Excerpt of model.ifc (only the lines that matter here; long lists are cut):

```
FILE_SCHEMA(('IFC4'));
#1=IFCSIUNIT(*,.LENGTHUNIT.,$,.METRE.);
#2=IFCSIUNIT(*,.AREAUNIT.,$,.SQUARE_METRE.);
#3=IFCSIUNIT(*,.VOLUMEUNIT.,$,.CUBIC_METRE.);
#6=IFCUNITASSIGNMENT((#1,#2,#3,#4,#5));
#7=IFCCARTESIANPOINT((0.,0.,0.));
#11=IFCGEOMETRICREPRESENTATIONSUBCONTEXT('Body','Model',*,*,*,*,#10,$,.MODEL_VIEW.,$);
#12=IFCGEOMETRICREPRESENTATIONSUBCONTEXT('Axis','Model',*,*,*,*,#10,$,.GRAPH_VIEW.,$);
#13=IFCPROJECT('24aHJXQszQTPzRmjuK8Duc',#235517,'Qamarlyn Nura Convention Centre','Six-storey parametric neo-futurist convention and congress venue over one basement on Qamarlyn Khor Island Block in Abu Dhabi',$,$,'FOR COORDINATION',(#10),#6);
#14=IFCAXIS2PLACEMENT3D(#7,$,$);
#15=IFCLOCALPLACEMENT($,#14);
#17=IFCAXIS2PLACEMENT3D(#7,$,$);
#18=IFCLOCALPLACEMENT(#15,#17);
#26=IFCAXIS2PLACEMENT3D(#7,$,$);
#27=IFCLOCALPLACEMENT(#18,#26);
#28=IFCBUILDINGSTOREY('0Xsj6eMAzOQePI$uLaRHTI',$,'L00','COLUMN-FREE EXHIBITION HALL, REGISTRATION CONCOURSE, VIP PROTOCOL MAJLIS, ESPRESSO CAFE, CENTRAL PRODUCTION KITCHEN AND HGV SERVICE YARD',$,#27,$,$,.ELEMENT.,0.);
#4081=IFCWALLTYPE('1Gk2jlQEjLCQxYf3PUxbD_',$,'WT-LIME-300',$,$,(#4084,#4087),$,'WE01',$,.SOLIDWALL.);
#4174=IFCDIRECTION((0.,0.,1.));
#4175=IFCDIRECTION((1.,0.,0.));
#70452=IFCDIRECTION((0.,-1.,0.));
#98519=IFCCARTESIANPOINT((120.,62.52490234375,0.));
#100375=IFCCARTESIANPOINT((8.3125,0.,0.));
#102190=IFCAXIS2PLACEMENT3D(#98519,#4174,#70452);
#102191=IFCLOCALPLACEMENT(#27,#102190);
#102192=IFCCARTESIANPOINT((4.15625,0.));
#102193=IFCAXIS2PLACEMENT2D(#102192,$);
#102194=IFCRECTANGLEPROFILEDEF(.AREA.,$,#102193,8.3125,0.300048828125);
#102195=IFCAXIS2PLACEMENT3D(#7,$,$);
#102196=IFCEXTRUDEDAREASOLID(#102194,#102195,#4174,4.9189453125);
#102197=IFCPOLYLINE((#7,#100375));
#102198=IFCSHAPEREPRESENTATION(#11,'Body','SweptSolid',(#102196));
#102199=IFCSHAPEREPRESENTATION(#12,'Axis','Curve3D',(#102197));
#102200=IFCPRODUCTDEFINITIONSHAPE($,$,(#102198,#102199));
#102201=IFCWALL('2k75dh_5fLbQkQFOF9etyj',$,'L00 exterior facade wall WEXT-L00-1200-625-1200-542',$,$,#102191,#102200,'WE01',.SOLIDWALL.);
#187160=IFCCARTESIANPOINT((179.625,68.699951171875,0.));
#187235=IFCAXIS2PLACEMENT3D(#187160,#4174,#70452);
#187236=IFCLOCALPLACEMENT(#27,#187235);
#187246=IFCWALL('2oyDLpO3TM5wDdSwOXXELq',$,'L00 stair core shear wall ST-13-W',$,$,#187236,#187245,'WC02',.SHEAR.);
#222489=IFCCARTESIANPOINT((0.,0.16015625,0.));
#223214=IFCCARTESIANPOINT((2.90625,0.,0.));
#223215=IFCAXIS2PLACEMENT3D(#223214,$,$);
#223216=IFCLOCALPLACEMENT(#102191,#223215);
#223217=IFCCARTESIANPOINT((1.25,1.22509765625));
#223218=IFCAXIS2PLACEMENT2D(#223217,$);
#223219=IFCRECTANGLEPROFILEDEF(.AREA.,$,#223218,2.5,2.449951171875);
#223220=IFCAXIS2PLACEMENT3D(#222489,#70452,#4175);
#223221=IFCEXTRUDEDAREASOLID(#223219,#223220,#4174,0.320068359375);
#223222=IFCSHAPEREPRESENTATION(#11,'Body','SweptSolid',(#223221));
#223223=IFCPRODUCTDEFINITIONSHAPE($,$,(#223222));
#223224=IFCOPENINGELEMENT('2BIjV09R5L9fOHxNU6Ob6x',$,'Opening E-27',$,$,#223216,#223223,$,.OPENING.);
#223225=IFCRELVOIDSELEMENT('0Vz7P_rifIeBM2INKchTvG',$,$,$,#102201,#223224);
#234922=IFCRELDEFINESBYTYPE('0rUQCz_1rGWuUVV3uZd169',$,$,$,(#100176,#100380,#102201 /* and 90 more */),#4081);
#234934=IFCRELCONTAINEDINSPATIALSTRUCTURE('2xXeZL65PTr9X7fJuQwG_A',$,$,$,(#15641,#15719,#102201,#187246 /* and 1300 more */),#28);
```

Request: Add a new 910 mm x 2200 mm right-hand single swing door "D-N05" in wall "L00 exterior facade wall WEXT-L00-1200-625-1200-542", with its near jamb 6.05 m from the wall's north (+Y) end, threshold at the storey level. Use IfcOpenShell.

```python
import numpy as np
import ifcopenshell
import ifcopenshell.api.feature
import ifcopenshell.api.geometry
import ifcopenshell.api.root
import ifcopenshell.api.spatial
import ifcopenshell.geom
import ifcopenshell.util.element
import ifcopenshell.util.placement
import ifcopenshell.util.representation
import ifcopenshell.util.shape
import ifcopenshell.util.unit

model = ifcopenshell.open("model.ifc")
unit_scale = ifcopenshell.util.unit.calculate_unit_scale(model)
settings = ifcopenshell.geom.settings()


def volume(element):
    """Net volume in cubic metres, openings subtracted."""
    shape = ifcopenshell.geom.create_shape(settings, element)
    return ifcopenshell.util.shape.get_volume(shape.geometry)


wall = model.by_id(102201)
storey = ifcopenshell.util.element.get_container(wall, ifc_class="IfcBuildingStorey")
context = ifcopenshell.util.representation.get_context(model, "Model", "Body", "MODEL_VIEW")
before = volume(wall)

width, height, from_end, sill = 0.91, 2.2, 6.05, 0.0  # metres

# The wall runs along its own X axis, and the end named is its -X end.
wall_shape = ifcopenshell.geom.create_shape(settings, wall)
x, y, z = ifcopenshell.util.shape.get_vertices(wall_shape.geometry).T
start = x.min() + from_end
face, thickness = float(y.min()), float(y.max() - y.min())
wall_matrix = ifcopenshell.util.placement.get_local_placement(wall.ObjectPlacement)
level = ifcopenshell.util.placement.get_local_placement(storey.ObjectPlacement)[2, 3]


def in_wall(x, y):
    """Placement at x, y metres in the wall's axes, at sill height."""
    matrix = wall_matrix.copy()
    matrix[:, 3] = wall_matrix @ np.array([x / unit_scale, y / unit_scale, 0.0, 1.0])
    matrix[2, 3] = level + sill / unit_scale
    return matrix


# Opening: a box that overshoots both wall faces by 50 mm.
opening = ifcopenshell.api.root.create_entity(model, ifc_class="IfcOpeningElement", predefined_type="OPENING")
box = ifcopenshell.api.geometry.add_wall_representation(
    model, context=context, length=width, height=height, thickness=thickness + 0.1
)
ifcopenshell.api.geometry.assign_representation(model, product=opening, representation=box)
ifcopenshell.api.geometry.edit_object_placement(model, product=opening, matrix=in_wall(start, face - 0.05), is_si=False)
ifcopenshell.api.feature.add_feature(model, feature=opening, element=wall)

door = ifcopenshell.api.root.create_entity(model, ifc_class="IfcDoor", name="D-N05", predefined_type="DOOR")
door.OverallWidth, door.OverallHeight = width / unit_scale, height / unit_scale
door.OperationType = "SINGLE_SWING_RIGHT"
body = ifcopenshell.api.geometry.add_door_representation(
    model,
    context=context,
    overall_width=door.OverallWidth,
    overall_height=door.OverallHeight,
    operation_type="SINGLE_SWING_RIGHT",
    lining_properties={"LiningDepth": thickness / unit_scale, "ThresholdDepth": thickness / unit_scale},
)
ifcopenshell.api.geometry.assign_representation(model, product=door, representation=body)
ifcopenshell.api.spatial.assign_container(model, products=[door], relating_structure=storey)
ifcopenshell.api.feature.add_filling(model, opening=opening, element=door)

# The lining spans the wall, so the door starts at the wall face.
ifcopenshell.api.geometry.edit_object_placement(model, product=door, matrix=in_wall(start, face), is_si=False)

after = volume(wall)

print(f"wall volume {before:.3f} -> {after:.3f} m3")

model.write("model_v2.ifc")
```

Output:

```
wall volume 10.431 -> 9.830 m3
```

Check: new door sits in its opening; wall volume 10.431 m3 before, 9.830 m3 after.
